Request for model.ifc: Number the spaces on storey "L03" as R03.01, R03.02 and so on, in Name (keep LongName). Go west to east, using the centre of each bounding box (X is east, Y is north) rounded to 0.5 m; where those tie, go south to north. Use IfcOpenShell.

First a look at what the model holds.

```python
import ifcopenshell
import ifcopenshell.util.element
import ifcopenshell.util.placement

model = ifcopenshell.open("model.ifc")
print(model.schema)
storey = next(s for s in model.by_type("IfcBuildingStorey") if s.Name == "L03")
spaces = [e for e in ifcopenshell.util.element.get_decomposition(storey) if e.is_a("IfcSpace")]
for e in sorted(spaces, key=lambda e: e.id()):
    origin = ifcopenshell.util.placement.get_local_placement(e.ObjectPlacement)[:3, 3]
    print(e.id(), e.Name, e.LongName, origin.round(2) + 0.0, sep=" | ")
```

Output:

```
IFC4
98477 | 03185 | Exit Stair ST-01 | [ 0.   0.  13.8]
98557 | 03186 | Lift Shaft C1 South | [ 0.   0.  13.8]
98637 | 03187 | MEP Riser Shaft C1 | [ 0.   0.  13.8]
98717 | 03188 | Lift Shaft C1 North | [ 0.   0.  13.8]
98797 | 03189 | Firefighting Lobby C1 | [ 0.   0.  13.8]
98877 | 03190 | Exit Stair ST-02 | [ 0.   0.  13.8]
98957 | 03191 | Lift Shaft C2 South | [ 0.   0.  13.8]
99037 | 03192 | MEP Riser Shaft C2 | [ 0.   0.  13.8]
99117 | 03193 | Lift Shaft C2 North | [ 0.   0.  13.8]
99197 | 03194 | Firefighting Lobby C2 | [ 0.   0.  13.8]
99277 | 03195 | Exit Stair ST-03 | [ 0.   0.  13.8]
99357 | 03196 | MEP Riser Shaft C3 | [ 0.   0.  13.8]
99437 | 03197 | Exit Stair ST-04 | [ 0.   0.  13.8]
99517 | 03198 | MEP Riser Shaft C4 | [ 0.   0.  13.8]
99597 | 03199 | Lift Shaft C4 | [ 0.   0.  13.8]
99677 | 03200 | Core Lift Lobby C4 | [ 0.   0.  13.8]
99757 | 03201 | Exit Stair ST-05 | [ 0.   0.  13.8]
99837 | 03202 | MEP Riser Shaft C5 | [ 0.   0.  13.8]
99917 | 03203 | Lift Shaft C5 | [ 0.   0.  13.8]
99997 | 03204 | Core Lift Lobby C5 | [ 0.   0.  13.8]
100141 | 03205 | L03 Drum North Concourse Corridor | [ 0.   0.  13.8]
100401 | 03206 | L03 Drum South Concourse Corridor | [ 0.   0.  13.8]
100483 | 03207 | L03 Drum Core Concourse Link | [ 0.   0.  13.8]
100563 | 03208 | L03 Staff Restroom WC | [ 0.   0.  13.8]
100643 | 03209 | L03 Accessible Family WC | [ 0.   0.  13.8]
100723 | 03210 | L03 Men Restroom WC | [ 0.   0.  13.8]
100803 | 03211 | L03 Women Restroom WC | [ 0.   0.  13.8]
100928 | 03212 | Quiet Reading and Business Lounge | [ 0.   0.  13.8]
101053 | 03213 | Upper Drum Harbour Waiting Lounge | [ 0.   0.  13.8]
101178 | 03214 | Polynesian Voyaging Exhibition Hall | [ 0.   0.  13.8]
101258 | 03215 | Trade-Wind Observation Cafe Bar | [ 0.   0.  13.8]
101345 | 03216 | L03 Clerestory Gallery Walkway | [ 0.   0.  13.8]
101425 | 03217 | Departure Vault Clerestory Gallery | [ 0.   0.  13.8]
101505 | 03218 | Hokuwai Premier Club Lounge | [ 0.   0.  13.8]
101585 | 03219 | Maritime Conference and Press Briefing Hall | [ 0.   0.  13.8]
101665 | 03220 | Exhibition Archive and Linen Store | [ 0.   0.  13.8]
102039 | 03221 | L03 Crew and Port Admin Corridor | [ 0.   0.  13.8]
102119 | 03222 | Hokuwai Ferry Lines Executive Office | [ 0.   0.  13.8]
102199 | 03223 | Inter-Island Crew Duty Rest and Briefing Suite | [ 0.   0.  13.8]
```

```python
import ifcopenshell
import ifcopenshell.geom
import ifcopenshell.util.element
import ifcopenshell.util.shape

model = ifcopenshell.open("model.ifc")
settings = ifcopenshell.geom.settings()
settings.set("use-world-coords", True)


def centre(element):
    shape = ifcopenshell.geom.create_shape(settings, element)
    return ifcopenshell.util.shape.get_bbox_centroid(shape.geometry)


storey = next(s for s in model.by_type("IfcBuildingStorey") if s.Name == "L03")
spaces = [e for e in ifcopenshell.util.element.get_decomposition(storey) if e.is_a("IfcSpace")]

# Insertion points can sit at a corner or the storey origin, so sort by the geometry (in metres).
centres = {e: centre(e) for e in spaces}
spaces.sort(key=lambda e: (round(centres[e][0] / 0.5), centres[e][1]))

for i, e in enumerate(spaces, start=1):
    number = f"R03.{i:02d}"
    e.Name = number
    print(e.id(), number)

model.write("model_v2.ifc")
```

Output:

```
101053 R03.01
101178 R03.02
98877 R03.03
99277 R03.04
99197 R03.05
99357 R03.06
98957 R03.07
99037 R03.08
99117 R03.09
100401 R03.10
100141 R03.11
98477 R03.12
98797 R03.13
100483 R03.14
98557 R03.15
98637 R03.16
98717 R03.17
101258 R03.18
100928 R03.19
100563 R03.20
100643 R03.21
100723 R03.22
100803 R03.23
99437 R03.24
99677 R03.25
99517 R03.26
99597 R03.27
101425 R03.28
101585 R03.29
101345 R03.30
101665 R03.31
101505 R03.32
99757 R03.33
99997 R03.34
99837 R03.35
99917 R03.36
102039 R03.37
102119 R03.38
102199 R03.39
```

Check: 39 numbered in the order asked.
